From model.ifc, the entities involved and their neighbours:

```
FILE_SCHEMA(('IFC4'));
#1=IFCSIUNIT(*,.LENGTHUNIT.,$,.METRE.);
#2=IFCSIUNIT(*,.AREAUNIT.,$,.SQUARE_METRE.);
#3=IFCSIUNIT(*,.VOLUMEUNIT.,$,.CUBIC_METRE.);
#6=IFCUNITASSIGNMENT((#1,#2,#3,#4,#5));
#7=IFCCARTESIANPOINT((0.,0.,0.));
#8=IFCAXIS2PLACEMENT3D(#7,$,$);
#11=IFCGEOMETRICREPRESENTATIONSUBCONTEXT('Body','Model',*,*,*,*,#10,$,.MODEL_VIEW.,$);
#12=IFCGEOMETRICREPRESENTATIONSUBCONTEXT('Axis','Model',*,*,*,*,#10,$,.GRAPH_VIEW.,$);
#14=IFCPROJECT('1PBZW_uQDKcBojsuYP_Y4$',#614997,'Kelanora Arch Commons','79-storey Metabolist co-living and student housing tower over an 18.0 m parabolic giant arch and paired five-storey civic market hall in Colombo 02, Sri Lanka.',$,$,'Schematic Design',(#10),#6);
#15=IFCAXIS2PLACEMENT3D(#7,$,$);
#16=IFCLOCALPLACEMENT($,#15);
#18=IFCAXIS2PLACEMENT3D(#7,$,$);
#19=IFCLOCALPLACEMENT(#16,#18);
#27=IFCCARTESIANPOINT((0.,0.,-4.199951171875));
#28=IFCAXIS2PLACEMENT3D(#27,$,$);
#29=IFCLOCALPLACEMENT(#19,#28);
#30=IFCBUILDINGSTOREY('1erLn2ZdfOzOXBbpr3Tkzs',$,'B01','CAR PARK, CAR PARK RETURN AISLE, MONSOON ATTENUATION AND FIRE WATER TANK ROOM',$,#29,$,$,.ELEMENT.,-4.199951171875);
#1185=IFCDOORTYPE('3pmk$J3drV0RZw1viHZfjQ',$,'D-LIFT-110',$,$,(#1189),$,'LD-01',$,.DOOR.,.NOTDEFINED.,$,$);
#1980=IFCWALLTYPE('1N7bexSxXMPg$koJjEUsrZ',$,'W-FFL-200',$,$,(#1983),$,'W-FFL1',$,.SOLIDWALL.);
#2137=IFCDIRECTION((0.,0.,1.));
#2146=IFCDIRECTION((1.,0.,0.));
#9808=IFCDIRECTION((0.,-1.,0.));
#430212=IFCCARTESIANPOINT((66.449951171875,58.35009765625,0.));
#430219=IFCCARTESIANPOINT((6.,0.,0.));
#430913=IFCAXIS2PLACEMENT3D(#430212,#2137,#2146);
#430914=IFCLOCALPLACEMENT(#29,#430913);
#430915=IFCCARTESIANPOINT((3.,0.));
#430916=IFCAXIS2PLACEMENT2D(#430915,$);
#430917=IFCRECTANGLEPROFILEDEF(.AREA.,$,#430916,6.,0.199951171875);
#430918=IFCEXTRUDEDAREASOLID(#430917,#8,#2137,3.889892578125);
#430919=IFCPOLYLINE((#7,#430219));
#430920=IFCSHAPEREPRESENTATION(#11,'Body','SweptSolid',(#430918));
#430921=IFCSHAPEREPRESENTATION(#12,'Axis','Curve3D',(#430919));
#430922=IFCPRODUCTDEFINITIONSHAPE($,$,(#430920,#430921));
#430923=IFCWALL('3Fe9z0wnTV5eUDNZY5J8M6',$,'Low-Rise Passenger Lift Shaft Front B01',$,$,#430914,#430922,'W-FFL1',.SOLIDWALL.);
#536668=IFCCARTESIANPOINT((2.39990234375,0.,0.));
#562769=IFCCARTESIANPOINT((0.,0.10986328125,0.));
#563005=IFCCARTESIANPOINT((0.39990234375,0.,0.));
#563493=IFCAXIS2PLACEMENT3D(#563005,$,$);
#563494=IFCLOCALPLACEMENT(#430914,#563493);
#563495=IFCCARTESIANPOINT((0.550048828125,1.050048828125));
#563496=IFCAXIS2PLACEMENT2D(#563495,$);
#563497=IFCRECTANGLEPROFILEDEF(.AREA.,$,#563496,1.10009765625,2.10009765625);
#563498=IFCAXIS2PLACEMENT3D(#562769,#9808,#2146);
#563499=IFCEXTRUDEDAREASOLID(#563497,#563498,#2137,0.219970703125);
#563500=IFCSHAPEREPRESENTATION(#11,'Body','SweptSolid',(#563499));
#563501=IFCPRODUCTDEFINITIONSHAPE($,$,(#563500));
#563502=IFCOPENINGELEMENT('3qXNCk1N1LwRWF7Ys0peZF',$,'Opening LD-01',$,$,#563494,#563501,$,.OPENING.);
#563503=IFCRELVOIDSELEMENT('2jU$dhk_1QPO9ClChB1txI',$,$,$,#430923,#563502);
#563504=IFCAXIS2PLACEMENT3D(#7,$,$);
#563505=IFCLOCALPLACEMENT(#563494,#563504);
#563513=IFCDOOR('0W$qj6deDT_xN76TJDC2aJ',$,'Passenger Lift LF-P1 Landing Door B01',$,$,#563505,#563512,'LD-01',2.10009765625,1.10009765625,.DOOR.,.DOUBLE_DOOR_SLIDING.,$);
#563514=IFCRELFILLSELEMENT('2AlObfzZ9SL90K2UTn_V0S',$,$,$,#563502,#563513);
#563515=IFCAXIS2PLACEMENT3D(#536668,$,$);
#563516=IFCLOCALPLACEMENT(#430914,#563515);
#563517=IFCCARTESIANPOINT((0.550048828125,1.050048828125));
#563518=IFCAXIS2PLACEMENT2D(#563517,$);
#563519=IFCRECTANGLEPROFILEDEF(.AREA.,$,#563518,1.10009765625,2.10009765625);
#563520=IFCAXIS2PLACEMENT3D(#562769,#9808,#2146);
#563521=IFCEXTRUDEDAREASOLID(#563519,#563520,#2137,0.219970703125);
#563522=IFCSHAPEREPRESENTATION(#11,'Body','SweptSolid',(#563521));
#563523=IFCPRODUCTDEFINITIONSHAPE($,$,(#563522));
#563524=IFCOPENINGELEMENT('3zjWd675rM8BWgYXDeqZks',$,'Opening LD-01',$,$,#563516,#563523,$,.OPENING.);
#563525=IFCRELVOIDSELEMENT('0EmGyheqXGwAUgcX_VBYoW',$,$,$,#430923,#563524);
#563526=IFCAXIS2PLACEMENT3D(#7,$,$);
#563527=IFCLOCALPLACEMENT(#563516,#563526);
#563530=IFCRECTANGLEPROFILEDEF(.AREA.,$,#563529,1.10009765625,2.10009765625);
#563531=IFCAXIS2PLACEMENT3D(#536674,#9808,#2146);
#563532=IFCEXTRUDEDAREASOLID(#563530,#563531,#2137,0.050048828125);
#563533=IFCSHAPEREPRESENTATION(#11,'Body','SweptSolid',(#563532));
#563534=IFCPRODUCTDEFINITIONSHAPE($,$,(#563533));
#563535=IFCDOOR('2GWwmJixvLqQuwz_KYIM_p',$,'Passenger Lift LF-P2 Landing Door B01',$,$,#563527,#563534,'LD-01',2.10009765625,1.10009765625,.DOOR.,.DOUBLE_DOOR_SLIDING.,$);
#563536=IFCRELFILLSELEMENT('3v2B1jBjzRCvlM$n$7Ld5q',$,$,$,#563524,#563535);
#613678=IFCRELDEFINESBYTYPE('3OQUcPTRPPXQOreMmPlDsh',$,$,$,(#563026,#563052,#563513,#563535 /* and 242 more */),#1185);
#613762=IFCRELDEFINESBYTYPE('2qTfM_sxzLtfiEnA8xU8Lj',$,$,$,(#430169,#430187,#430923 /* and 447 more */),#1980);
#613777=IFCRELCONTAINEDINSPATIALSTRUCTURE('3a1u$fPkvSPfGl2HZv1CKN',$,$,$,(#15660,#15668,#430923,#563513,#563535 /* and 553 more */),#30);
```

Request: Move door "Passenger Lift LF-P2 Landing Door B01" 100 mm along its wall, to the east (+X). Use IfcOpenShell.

```python
import ifcopenshell
import ifcopenshell.api.geometry
import ifcopenshell.util.placement

model = ifcopenshell.open("model.ifc")

door = model.by_guid("2GWwmJixvLqQuwz_KYIM_p")
opening = door.FillsVoids[0].RelatingOpeningElement
wall = opening.VoidsElements[0].RelatingBuildingElement

wall_matrix = ifcopenshell.util.placement.get_local_placement(wall.ObjectPlacement)
shift = wall_matrix[:3, 0] * 0.1
before = ifcopenshell.util.placement.get_local_placement(door.ObjectPlacement)[:3, 3].copy()

# The door is placed relative to its opening, so it follows when the opening moves.
matrix = ifcopenshell.util.placement.get_local_placement(opening.ObjectPlacement)
matrix[:3, 3] += shift
ifcopenshell.api.geometry.edit_object_placement(
    model, product=opening, matrix=matrix, is_si=False, should_transform_children=True
)

after = ifcopenshell.util.placement.get_local_placement(door.ObjectPlacement)[:3, 3]
print("door moved by", (after - before).round(3) + 0.0)

model.write("model_rev.ifc")
```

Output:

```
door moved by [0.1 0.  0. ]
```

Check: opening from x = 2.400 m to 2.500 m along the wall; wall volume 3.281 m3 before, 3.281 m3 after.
